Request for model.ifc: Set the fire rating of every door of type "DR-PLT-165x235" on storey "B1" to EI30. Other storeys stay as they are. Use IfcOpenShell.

First a look at what the model holds.

```python
import ifcopenshell
import ifcopenshell.util.element

model = ifcopenshell.open("model.ifc")
print(model.schema)
storey = next(s for s in model.by_type("IfcBuildingStorey") if s.Name == "B1")
doors = [e for e in ifcopenshell.util.element.get_decomposition(storey) if e.is_a("IfcDoor")]
seen = {}
for e in doors:
    element_type = ifcopenshell.util.element.get_type(e)
    key = (element_type.Name if element_type != e and element_type else None, ifcopenshell.util.element.get_pset(e, "Pset_DoorCommon", "FireRating"))
    seen[key] = seen.get(key, 0) + 1
for (name, value), count in sorted(seen.items(), key=str):
    print(count, "x", name, "|", value)
```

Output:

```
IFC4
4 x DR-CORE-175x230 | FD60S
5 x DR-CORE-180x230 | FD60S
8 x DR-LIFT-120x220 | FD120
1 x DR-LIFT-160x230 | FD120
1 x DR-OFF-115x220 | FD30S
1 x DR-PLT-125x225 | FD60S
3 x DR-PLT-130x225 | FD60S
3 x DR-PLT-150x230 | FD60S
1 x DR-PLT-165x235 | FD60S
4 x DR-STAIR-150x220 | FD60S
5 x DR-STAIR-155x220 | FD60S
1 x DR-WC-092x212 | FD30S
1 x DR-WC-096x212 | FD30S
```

```python
import ifcopenshell
import ifcopenshell.api.pset
import ifcopenshell.util.element

model = ifcopenshell.open("model.ifc")

storey = next(s for s in model.by_type("IfcBuildingStorey") if s.Name == "B1")
doors = [e for e in ifcopenshell.util.element.get_decomposition(storey) if e.is_a("IfcDoor")]

count = 0
for e in doors:
    element_type = ifcopenshell.util.element.get_type(e)
    if element_type in (None, e) or element_type.Name != "DR-PLT-165x235":
        continue
    # add_pset returns the element's existing set when there is one.
    pset = ifcopenshell.api.pset.add_pset(model, product=e, name="Pset_DoorCommon")
    ifcopenshell.api.pset.edit_pset(model, pset=pset, properties={"FireRating": "EI30"})
    count += 1

print(count, "doors updated")

model.write("model_v2.ifc")
```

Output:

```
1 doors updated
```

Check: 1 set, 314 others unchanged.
